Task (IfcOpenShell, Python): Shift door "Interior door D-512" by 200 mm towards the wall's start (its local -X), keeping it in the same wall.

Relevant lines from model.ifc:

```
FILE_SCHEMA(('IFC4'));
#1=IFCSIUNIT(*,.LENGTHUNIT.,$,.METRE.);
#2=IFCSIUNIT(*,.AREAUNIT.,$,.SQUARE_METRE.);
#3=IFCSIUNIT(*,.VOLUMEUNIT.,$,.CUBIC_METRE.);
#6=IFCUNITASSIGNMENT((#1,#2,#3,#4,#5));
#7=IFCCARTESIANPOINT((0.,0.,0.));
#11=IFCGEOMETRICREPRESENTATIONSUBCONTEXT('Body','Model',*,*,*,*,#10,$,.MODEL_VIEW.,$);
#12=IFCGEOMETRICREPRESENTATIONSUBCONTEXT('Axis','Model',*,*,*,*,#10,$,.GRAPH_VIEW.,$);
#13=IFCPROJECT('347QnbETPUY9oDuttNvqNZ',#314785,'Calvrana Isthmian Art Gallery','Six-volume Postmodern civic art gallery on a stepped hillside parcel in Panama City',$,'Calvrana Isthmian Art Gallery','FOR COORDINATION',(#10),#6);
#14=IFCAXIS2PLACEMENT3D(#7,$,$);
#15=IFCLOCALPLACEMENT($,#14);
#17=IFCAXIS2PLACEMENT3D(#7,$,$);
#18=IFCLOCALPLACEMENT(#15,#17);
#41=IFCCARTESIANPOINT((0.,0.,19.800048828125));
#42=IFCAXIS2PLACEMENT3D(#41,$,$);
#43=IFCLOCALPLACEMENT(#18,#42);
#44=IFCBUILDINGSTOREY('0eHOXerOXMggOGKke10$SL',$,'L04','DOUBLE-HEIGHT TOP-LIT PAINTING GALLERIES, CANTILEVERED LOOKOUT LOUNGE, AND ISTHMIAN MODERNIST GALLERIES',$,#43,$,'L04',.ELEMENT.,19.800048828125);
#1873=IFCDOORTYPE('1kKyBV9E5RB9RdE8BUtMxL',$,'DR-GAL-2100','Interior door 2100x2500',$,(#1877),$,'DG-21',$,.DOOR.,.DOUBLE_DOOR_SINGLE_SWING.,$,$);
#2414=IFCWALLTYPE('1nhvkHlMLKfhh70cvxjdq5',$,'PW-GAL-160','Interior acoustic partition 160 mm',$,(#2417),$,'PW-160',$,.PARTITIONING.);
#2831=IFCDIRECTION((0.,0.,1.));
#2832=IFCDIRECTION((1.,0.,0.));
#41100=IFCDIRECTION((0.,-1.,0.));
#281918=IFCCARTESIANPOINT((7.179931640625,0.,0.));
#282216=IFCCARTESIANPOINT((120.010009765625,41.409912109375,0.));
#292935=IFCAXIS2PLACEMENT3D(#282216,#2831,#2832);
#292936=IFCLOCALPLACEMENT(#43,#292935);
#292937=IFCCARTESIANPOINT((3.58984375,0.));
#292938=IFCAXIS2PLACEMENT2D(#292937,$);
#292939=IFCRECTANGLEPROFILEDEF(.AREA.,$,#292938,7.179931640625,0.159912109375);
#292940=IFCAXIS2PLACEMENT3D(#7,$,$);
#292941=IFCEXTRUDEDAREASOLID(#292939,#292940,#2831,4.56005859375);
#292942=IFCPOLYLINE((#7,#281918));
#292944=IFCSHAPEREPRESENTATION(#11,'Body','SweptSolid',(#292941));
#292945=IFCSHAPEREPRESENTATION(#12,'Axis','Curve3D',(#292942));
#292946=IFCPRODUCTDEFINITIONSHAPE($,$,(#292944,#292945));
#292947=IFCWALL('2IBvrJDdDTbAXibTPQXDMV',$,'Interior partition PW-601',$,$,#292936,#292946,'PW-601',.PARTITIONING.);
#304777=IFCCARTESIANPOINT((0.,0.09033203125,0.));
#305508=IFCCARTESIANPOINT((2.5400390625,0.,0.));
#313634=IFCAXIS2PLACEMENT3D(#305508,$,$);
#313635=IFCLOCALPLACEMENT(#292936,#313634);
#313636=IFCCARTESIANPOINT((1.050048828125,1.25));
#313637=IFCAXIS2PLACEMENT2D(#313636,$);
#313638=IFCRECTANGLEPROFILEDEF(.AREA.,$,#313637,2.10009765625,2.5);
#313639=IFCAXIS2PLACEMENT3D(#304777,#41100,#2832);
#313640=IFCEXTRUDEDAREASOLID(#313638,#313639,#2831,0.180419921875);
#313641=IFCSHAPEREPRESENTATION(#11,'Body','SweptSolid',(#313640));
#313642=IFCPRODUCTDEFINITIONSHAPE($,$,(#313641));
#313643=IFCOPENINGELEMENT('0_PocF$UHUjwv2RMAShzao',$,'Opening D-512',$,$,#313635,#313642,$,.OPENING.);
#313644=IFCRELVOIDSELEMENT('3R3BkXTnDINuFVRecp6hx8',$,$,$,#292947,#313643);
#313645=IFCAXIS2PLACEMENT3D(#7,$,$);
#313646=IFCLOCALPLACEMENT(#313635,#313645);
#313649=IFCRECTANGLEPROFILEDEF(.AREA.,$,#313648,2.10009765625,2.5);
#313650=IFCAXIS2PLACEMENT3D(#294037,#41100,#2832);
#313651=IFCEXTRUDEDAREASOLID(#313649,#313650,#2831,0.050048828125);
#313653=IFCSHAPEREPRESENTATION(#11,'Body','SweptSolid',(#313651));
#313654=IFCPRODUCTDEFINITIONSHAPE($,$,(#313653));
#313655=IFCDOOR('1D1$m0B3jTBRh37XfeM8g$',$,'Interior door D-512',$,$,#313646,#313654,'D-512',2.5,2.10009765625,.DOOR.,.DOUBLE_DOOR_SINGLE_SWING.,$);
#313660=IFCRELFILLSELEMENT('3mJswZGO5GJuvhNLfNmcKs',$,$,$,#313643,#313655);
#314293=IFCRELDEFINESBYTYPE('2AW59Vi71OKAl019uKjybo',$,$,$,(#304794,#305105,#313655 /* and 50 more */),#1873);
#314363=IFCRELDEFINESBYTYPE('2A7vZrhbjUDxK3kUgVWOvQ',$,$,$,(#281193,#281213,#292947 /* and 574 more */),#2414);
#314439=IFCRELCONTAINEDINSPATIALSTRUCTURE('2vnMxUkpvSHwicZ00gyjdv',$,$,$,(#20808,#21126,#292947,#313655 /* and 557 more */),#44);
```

```python
import ifcopenshell
import ifcopenshell.api.geometry
import ifcopenshell.util.placement

model = ifcopenshell.open("model.ifc")

door = model.by_guid("1D1$m0B3jTBRh37XfeM8g$")
opening = door.FillsVoids[0].RelatingOpeningElement
wall = opening.VoidsElements[0].RelatingBuildingElement

wall_matrix = ifcopenshell.util.placement.get_local_placement(wall.ObjectPlacement)
shift = wall_matrix[:3, 0] * -0.2
before = ifcopenshell.util.placement.get_local_placement(door.ObjectPlacement)[:3, 3].copy()

# The door is placed relative to its opening, so it follows when the opening moves.
matrix = ifcopenshell.util.placement.get_local_placement(opening.ObjectPlacement)
matrix[:3, 3] += shift
ifcopenshell.api.geometry.edit_object_placement(
    model, product=opening, matrix=matrix, is_si=False, should_transform_children=True
)

after = ifcopenshell.util.placement.get_local_placement(door.ObjectPlacement)[:3, 3]
print("door moved by", (after - before).round(3) + 0.0)

model.write("model_v2.ifc")
```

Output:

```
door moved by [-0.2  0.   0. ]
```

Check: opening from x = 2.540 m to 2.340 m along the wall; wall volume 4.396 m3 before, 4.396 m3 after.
